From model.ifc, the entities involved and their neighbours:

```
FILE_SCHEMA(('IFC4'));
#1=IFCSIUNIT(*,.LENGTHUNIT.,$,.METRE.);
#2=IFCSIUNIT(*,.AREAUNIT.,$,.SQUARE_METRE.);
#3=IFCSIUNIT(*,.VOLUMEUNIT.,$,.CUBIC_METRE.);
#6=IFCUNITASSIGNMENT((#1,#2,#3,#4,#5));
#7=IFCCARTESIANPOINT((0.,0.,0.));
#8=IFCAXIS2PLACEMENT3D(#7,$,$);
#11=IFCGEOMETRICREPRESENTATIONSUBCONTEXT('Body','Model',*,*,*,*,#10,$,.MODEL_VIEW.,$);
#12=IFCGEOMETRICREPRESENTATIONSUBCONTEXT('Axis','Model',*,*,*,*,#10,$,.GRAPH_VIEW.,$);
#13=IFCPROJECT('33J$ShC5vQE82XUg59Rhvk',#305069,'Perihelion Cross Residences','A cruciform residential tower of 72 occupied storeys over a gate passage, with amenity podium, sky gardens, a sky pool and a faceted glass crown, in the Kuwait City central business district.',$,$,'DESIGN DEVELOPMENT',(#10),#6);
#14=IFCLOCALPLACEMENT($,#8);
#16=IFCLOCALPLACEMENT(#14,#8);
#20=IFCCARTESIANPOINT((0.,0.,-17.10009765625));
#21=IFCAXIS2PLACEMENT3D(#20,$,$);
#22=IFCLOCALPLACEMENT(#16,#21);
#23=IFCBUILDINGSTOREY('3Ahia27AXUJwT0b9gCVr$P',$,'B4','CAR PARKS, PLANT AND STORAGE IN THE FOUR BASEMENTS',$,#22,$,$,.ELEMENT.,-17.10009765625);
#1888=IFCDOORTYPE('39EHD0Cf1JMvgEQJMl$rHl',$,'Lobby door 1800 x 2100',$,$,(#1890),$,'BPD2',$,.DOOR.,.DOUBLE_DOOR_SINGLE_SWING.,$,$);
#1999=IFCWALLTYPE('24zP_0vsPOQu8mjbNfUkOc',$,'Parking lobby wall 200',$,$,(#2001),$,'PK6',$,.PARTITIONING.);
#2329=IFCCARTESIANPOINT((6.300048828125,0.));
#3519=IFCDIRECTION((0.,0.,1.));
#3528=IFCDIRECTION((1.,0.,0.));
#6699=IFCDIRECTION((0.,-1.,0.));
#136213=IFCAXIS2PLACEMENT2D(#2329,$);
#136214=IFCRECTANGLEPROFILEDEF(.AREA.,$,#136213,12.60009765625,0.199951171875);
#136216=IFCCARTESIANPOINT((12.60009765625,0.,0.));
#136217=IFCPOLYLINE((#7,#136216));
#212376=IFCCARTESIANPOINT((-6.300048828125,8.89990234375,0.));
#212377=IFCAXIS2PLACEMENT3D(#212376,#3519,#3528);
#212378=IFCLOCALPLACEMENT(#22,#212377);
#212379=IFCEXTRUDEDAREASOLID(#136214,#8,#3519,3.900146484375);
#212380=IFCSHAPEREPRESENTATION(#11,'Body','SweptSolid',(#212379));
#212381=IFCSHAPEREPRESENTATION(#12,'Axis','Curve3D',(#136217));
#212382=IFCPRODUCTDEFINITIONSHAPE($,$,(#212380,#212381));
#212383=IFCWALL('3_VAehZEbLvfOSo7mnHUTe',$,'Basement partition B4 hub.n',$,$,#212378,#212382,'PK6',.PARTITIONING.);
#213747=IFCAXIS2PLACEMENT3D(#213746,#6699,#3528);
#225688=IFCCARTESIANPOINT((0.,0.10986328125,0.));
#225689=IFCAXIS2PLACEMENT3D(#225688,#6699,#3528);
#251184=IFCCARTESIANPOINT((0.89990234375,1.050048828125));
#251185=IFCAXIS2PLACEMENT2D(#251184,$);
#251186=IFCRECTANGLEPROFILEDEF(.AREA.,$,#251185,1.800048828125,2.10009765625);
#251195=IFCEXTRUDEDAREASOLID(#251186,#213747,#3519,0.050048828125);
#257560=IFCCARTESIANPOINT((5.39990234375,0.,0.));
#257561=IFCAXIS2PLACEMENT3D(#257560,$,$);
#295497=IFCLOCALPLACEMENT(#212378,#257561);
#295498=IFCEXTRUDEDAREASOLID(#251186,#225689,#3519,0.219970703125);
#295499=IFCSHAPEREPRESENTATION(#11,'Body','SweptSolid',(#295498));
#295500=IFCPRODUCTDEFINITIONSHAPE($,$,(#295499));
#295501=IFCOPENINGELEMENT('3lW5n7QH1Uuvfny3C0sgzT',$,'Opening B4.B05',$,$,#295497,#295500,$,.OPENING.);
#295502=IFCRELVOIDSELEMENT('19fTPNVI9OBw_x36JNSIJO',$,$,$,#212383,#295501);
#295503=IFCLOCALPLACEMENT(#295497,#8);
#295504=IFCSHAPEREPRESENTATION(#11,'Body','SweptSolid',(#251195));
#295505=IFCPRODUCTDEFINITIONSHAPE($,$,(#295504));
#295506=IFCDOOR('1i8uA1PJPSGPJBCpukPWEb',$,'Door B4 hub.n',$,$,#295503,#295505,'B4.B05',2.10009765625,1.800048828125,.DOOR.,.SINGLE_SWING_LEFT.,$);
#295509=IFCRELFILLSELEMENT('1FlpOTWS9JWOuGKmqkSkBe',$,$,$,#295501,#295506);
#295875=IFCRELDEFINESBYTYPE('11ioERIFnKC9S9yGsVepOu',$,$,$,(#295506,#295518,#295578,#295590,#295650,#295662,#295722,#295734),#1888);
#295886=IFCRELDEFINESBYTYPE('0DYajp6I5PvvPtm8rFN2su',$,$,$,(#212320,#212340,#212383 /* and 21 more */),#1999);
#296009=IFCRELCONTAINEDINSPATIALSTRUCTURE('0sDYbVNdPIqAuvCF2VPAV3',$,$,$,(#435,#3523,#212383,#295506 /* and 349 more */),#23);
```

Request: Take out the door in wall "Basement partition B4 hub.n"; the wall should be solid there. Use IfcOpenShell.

```python
import ifcopenshell
import ifcopenshell.api.feature
import ifcopenshell.api.root
import ifcopenshell.geom
import ifcopenshell.util.shape

model = ifcopenshell.open("model.ifc")
settings = ifcopenshell.geom.settings()


def volume(element):
    """Net volume in cubic metres, openings subtracted."""
    shape = ifcopenshell.geom.create_shape(settings, element)
    return ifcopenshell.util.shape.get_volume(shape.geometry)


door = model.by_guid("1i8uA1PJPSGPJBCpukPWEb")
opening = door.FillsVoids[0].RelatingOpeningElement
wall = opening.VoidsElements[0].RelatingBuildingElement
before = volume(wall)

ifcopenshell.api.root.remove_product(model, product=door)
ifcopenshell.api.feature.remove_feature(model, feature=opening)

after = volume(wall)

print(f"wall volume {before:.3f} -> {after:.3f} m3")

model.write("model_v2.ifc")
```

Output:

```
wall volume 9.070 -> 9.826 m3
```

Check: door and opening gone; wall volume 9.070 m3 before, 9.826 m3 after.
